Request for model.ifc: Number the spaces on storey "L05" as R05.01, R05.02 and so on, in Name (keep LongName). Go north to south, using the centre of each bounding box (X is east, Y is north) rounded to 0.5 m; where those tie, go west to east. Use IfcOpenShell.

First a look at what the model holds.

```python
import ifcopenshell
import ifcopenshell.util.element
import ifcopenshell.util.placement

model = ifcopenshell.open("model.ifc")
print(model.schema)
storey = next(s for s in model.by_type("IfcBuildingStorey") if s.Name == "L05")
spaces = [e for e in ifcopenshell.util.element.get_decomposition(storey) if e.is_a("IfcSpace")]
for e in sorted(spaces, key=lambda e: e.id()):
    origin = ifcopenshell.util.placement.get_local_placement(e.ObjectPlacement)[:3, 3]
    print(e.id(), e.Name, e.LongName, origin.round(2) + 0.0, sep=" | ")
```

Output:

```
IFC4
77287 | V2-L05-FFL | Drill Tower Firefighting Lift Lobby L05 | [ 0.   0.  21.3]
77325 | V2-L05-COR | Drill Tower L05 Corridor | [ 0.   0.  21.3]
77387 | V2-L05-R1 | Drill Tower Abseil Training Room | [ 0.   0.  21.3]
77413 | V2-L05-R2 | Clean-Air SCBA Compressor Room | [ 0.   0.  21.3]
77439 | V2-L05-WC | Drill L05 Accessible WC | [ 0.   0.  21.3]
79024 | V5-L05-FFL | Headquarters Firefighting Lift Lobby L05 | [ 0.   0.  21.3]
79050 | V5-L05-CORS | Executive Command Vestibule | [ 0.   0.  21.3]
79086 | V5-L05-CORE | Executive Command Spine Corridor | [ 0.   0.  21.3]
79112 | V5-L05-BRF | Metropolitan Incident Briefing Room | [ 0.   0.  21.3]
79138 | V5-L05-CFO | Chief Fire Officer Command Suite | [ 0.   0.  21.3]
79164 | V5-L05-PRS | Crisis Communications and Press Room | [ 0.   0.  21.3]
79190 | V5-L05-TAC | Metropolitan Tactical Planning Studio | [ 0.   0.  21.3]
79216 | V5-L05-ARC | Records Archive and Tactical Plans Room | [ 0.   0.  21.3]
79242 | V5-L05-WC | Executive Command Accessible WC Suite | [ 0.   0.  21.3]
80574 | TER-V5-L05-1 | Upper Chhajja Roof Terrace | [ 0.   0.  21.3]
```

```python
import ifcopenshell
import ifcopenshell.geom
import ifcopenshell.util.element
import ifcopenshell.util.shape

model = ifcopenshell.open("model.ifc")
settings = ifcopenshell.geom.settings()
settings.set("use-world-coords", True)


def centre(element):
    shape = ifcopenshell.geom.create_shape(settings, element)
    return ifcopenshell.util.shape.get_bbox_centroid(shape.geometry)


storey = next(s for s in model.by_type("IfcBuildingStorey") if s.Name == "L05")
spaces = [e for e in ifcopenshell.util.element.get_decomposition(storey) if e.is_a("IfcSpace")]

# Insertion points can sit at a corner or the storey origin, so sort by the geometry (in metres).
centres = {e: centre(e) for e in spaces}
spaces.sort(key=lambda e: (-round(centres[e][1] / 0.5), centres[e][0]))

for i, e in enumerate(spaces, start=1):
    number = f"R05.{i:02d}"
    e.Name = number
    print(e.id(), number)

model.write("model_updated.ifc")
```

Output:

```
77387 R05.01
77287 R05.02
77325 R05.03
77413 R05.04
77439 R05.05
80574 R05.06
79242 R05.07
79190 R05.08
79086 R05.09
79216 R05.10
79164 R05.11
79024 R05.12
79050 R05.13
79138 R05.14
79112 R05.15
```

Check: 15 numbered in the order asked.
